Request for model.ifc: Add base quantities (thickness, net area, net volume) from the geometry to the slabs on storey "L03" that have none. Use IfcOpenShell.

First a look at what the model holds.

```python
import ifcopenshell
import ifcopenshell.util.element
import ifcopenshell.util.unit

model = ifcopenshell.open("model.ifc")
print(model.schema)
for unit_type in ("LENGTHUNIT", "AREAUNIT", "VOLUMEUNIT"):
    print(unit_type, ifcopenshell.util.unit.calculate_unit_scale(model, unit_type))
storey = next(s for s in model.by_type("IfcBuildingStorey") if s.Name == "L03")
slabs = [e for e in ifcopenshell.util.element.get_decomposition(storey) if e.is_a("IfcSlab")]
for e in sorted(slabs, key=lambda e: e.id()):
    print(e.id(), e.is_a(), e.Name, list(ifcopenshell.util.element.get_psets(e, qtos_only=True)), sep=" | ")
```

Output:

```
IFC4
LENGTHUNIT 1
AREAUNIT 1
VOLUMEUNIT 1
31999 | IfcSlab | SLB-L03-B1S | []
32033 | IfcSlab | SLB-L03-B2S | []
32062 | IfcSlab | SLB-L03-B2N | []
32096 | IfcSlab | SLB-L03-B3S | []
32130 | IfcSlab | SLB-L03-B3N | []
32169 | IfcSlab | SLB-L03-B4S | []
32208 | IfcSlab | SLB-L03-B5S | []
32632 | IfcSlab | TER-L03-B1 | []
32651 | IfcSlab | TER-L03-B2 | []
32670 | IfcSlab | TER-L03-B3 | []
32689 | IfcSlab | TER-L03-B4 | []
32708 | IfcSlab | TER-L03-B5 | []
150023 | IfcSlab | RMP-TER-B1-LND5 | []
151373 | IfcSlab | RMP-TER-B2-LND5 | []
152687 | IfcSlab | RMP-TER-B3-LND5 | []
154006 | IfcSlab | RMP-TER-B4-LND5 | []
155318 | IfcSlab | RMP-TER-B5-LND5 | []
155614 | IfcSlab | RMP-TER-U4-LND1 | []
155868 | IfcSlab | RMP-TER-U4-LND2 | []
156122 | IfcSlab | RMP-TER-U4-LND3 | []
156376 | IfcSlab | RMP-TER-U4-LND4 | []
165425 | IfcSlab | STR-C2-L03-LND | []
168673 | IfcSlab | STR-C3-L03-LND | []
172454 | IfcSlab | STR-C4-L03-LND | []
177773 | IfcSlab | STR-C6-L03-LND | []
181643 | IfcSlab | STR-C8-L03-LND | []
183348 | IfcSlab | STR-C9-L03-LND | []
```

```python
import ifcopenshell
import ifcopenshell.api.pset
import ifcopenshell.geom
import ifcopenshell.util.element
import ifcopenshell.util.shape
import ifcopenshell.util.unit

model = ifcopenshell.open("model.ifc")
unit_scale = ifcopenshell.util.unit.calculate_unit_scale(model)
area_scale = ifcopenshell.util.unit.calculate_unit_scale(model, "AREAUNIT")
volume_scale = ifcopenshell.util.unit.calculate_unit_scale(model, "VOLUMEUNIT")
settings = ifcopenshell.geom.settings()

storey = next(s for s in model.by_type("IfcBuildingStorey") if s.Name == "L03")
slabs = [e for e in ifcopenshell.util.element.get_decomposition(storey) if e.is_a("IfcSlab")]

for e in sorted(slabs, key=lambda e: e.id()):
    if ifcopenshell.util.element.get_psets(e, qtos_only=True, should_inherit=False):
        continue
    # Geometry comes back in metres, in the element's own axes.
    shape = ifcopenshell.geom.create_shape(settings, e)
    values = {
        "Width": ifcopenshell.util.shape.get_z(shape.geometry) / unit_scale,
        "NetArea": ifcopenshell.util.shape.get_footprint_area(shape.geometry) / area_scale,
        "NetVolume": ifcopenshell.util.shape.get_volume(shape.geometry) / volume_scale,
    }
    qto = ifcopenshell.api.pset.add_qto(model, product=e, name="Qto_SlabBaseQuantities")
    ifcopenshell.api.pset.edit_qto(model, qto=qto, properties=values)
    print(e.id(), {k: round(v, 3) for k, v in values.items()})

model.write("model_edited.ifc")
```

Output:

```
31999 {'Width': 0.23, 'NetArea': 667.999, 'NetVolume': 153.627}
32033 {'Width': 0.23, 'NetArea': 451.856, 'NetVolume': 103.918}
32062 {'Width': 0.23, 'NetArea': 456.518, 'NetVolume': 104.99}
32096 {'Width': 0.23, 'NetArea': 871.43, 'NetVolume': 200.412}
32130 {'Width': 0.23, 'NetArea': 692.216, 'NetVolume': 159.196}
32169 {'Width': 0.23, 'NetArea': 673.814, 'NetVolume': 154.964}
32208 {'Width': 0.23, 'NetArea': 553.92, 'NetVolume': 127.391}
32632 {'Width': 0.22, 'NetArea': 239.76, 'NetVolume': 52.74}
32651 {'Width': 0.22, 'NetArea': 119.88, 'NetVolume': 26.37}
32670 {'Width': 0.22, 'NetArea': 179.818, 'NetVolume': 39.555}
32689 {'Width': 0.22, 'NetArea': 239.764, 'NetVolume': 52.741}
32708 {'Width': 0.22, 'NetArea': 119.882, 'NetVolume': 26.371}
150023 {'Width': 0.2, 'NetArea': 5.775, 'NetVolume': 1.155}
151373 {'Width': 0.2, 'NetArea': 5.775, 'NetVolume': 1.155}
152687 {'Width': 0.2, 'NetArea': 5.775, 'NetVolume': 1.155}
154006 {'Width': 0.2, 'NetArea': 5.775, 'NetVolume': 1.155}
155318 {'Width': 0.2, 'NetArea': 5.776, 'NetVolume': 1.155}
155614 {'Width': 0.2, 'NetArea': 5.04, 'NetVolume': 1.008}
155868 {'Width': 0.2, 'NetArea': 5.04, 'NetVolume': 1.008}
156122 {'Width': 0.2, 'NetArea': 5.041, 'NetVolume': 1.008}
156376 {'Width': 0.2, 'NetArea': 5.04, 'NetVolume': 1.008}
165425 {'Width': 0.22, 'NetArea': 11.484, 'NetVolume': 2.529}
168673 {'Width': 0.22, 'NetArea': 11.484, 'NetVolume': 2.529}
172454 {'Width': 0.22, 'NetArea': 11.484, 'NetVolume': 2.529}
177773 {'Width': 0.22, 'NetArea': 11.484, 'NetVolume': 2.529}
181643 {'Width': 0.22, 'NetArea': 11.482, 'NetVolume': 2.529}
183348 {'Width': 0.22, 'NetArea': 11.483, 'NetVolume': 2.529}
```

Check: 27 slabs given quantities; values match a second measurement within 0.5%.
